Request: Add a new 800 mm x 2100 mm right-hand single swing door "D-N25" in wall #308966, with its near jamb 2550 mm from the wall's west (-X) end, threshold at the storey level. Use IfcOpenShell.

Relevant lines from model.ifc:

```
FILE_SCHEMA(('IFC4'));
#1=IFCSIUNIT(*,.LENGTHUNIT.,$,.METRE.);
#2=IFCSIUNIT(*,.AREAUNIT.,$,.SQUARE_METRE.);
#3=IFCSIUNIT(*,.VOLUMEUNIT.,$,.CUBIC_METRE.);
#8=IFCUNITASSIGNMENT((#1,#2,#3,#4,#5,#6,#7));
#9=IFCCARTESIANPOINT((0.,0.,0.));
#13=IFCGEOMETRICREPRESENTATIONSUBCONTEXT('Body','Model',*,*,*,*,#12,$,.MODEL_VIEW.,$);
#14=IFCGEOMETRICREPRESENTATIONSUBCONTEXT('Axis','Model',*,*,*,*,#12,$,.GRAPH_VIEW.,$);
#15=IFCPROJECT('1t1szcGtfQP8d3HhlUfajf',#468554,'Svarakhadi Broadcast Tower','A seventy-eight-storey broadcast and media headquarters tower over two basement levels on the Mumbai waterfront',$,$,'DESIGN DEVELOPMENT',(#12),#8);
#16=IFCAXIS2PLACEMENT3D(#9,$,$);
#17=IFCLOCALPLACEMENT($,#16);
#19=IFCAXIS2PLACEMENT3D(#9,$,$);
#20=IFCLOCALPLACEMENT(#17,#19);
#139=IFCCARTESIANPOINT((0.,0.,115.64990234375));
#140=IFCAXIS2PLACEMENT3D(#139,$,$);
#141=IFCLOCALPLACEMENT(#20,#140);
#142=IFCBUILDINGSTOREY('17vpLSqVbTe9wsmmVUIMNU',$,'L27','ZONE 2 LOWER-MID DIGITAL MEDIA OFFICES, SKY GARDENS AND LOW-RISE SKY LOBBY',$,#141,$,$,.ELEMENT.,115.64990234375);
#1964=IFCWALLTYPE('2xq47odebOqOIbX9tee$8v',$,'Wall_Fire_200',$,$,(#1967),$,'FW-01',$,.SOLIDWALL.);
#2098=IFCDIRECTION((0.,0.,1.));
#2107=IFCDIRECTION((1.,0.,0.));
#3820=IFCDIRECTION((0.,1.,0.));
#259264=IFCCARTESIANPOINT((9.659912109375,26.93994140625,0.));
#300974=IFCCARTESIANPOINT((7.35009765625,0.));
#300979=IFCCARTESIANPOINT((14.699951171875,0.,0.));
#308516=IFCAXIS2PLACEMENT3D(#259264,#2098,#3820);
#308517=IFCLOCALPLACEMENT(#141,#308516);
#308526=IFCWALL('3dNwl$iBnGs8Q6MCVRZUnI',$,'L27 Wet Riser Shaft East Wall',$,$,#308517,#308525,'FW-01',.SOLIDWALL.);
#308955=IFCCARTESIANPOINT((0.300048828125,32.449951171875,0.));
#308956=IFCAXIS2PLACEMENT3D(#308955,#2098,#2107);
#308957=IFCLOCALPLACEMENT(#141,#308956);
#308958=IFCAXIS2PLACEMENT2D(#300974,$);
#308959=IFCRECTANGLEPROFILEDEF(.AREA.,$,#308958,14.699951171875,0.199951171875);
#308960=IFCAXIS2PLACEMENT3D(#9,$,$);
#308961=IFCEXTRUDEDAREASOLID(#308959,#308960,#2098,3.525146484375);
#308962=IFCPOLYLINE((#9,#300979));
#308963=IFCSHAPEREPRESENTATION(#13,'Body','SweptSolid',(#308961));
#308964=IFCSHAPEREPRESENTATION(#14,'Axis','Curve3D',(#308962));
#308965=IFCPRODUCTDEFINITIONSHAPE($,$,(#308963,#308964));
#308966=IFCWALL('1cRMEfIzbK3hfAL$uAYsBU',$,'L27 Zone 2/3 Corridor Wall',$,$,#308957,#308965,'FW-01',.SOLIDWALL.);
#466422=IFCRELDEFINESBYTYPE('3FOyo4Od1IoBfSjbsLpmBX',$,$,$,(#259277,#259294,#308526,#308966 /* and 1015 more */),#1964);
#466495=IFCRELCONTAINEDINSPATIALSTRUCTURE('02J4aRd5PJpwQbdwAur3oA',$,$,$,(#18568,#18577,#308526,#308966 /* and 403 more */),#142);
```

```python
import numpy as np
import ifcopenshell
import ifcopenshell.api.feature
import ifcopenshell.api.geometry
import ifcopenshell.api.root
import ifcopenshell.api.spatial
import ifcopenshell.geom
import ifcopenshell.util.element
import ifcopenshell.util.placement
import ifcopenshell.util.representation
import ifcopenshell.util.shape
import ifcopenshell.util.unit

model = ifcopenshell.open("model.ifc")
unit_scale = ifcopenshell.util.unit.calculate_unit_scale(model)
settings = ifcopenshell.geom.settings()


def volume(element):
    """Net volume in cubic metres, openings subtracted."""
    shape = ifcopenshell.geom.create_shape(settings, element)
    return ifcopenshell.util.shape.get_volume(shape.geometry)


wall = model.by_id(308966)
storey = ifcopenshell.util.element.get_container(wall, ifc_class="IfcBuildingStorey")
context = ifcopenshell.util.representation.get_context(model, "Model", "Body", "MODEL_VIEW")
before = volume(wall)

width, height, from_end, sill = 0.8, 2.1, 2.55, 0.0  # metres

# The wall runs along its own X axis, and the end named is its -X end.
wall_shape = ifcopenshell.geom.create_shape(settings, wall)
x, y, z = ifcopenshell.util.shape.get_vertices(wall_shape.geometry).T
start = x.min() + from_end
face, thickness = float(y.min()), float(y.max() - y.min())
wall_matrix = ifcopenshell.util.placement.get_local_placement(wall.ObjectPlacement)
level = ifcopenshell.util.placement.get_local_placement(storey.ObjectPlacement)[2, 3]


def in_wall(x, y):
    """Placement at x, y metres in the wall's axes, at sill height."""
    matrix = wall_matrix.copy()
    matrix[:, 3] = wall_matrix @ np.array([x / unit_scale, y / unit_scale, 0.0, 1.0])
    matrix[2, 3] = level + sill / unit_scale
    return matrix


# Opening: a box that overshoots both wall faces by 50 mm.
opening = ifcopenshell.api.root.create_entity(model, ifc_class="IfcOpeningElement", predefined_type="OPENING")
box = ifcopenshell.api.geometry.add_wall_representation(
    model, context=context, length=width, height=height, thickness=thickness + 0.1
)
ifcopenshell.api.geometry.assign_representation(model, product=opening, representation=box)
ifcopenshell.api.geometry.edit_object_placement(model, product=opening, matrix=in_wall(start, face - 0.05), is_si=False)
ifcopenshell.api.feature.add_feature(model, feature=opening, element=wall)

door = ifcopenshell.api.root.create_entity(model, ifc_class="IfcDoor", name="D-N25", predefined_type="DOOR")
door.OverallWidth, door.OverallHeight = width / unit_scale, height / unit_scale
door.OperationType = "SINGLE_SWING_RIGHT"
body = ifcopenshell.api.geometry.add_door_representation(
    model,
    context=context,
    overall_width=door.OverallWidth,
    overall_height=door.OverallHeight,
    operation_type="SINGLE_SWING_RIGHT",
    lining_properties={"LiningDepth": thickness / unit_scale, "ThresholdDepth": thickness / unit_scale},
)
ifcopenshell.api.geometry.assign_representation(model, product=door, representation=body)
ifcopenshell.api.spatial.assign_container(model, products=[door], relating_structure=storey)
ifcopenshell.api.feature.add_filling(model, opening=opening, element=door)

# The lining spans the wall, so the door starts at the wall face.
ifcopenshell.api.geometry.edit_object_placement(model, product=door, matrix=in_wall(start, face), is_si=False)

after = volume(wall)

print(f"wall volume {before:.3f} -> {after:.3f} m3")

model.write("model_rev.ifc")
```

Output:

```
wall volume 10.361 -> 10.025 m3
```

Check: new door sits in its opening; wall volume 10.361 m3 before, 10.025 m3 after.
